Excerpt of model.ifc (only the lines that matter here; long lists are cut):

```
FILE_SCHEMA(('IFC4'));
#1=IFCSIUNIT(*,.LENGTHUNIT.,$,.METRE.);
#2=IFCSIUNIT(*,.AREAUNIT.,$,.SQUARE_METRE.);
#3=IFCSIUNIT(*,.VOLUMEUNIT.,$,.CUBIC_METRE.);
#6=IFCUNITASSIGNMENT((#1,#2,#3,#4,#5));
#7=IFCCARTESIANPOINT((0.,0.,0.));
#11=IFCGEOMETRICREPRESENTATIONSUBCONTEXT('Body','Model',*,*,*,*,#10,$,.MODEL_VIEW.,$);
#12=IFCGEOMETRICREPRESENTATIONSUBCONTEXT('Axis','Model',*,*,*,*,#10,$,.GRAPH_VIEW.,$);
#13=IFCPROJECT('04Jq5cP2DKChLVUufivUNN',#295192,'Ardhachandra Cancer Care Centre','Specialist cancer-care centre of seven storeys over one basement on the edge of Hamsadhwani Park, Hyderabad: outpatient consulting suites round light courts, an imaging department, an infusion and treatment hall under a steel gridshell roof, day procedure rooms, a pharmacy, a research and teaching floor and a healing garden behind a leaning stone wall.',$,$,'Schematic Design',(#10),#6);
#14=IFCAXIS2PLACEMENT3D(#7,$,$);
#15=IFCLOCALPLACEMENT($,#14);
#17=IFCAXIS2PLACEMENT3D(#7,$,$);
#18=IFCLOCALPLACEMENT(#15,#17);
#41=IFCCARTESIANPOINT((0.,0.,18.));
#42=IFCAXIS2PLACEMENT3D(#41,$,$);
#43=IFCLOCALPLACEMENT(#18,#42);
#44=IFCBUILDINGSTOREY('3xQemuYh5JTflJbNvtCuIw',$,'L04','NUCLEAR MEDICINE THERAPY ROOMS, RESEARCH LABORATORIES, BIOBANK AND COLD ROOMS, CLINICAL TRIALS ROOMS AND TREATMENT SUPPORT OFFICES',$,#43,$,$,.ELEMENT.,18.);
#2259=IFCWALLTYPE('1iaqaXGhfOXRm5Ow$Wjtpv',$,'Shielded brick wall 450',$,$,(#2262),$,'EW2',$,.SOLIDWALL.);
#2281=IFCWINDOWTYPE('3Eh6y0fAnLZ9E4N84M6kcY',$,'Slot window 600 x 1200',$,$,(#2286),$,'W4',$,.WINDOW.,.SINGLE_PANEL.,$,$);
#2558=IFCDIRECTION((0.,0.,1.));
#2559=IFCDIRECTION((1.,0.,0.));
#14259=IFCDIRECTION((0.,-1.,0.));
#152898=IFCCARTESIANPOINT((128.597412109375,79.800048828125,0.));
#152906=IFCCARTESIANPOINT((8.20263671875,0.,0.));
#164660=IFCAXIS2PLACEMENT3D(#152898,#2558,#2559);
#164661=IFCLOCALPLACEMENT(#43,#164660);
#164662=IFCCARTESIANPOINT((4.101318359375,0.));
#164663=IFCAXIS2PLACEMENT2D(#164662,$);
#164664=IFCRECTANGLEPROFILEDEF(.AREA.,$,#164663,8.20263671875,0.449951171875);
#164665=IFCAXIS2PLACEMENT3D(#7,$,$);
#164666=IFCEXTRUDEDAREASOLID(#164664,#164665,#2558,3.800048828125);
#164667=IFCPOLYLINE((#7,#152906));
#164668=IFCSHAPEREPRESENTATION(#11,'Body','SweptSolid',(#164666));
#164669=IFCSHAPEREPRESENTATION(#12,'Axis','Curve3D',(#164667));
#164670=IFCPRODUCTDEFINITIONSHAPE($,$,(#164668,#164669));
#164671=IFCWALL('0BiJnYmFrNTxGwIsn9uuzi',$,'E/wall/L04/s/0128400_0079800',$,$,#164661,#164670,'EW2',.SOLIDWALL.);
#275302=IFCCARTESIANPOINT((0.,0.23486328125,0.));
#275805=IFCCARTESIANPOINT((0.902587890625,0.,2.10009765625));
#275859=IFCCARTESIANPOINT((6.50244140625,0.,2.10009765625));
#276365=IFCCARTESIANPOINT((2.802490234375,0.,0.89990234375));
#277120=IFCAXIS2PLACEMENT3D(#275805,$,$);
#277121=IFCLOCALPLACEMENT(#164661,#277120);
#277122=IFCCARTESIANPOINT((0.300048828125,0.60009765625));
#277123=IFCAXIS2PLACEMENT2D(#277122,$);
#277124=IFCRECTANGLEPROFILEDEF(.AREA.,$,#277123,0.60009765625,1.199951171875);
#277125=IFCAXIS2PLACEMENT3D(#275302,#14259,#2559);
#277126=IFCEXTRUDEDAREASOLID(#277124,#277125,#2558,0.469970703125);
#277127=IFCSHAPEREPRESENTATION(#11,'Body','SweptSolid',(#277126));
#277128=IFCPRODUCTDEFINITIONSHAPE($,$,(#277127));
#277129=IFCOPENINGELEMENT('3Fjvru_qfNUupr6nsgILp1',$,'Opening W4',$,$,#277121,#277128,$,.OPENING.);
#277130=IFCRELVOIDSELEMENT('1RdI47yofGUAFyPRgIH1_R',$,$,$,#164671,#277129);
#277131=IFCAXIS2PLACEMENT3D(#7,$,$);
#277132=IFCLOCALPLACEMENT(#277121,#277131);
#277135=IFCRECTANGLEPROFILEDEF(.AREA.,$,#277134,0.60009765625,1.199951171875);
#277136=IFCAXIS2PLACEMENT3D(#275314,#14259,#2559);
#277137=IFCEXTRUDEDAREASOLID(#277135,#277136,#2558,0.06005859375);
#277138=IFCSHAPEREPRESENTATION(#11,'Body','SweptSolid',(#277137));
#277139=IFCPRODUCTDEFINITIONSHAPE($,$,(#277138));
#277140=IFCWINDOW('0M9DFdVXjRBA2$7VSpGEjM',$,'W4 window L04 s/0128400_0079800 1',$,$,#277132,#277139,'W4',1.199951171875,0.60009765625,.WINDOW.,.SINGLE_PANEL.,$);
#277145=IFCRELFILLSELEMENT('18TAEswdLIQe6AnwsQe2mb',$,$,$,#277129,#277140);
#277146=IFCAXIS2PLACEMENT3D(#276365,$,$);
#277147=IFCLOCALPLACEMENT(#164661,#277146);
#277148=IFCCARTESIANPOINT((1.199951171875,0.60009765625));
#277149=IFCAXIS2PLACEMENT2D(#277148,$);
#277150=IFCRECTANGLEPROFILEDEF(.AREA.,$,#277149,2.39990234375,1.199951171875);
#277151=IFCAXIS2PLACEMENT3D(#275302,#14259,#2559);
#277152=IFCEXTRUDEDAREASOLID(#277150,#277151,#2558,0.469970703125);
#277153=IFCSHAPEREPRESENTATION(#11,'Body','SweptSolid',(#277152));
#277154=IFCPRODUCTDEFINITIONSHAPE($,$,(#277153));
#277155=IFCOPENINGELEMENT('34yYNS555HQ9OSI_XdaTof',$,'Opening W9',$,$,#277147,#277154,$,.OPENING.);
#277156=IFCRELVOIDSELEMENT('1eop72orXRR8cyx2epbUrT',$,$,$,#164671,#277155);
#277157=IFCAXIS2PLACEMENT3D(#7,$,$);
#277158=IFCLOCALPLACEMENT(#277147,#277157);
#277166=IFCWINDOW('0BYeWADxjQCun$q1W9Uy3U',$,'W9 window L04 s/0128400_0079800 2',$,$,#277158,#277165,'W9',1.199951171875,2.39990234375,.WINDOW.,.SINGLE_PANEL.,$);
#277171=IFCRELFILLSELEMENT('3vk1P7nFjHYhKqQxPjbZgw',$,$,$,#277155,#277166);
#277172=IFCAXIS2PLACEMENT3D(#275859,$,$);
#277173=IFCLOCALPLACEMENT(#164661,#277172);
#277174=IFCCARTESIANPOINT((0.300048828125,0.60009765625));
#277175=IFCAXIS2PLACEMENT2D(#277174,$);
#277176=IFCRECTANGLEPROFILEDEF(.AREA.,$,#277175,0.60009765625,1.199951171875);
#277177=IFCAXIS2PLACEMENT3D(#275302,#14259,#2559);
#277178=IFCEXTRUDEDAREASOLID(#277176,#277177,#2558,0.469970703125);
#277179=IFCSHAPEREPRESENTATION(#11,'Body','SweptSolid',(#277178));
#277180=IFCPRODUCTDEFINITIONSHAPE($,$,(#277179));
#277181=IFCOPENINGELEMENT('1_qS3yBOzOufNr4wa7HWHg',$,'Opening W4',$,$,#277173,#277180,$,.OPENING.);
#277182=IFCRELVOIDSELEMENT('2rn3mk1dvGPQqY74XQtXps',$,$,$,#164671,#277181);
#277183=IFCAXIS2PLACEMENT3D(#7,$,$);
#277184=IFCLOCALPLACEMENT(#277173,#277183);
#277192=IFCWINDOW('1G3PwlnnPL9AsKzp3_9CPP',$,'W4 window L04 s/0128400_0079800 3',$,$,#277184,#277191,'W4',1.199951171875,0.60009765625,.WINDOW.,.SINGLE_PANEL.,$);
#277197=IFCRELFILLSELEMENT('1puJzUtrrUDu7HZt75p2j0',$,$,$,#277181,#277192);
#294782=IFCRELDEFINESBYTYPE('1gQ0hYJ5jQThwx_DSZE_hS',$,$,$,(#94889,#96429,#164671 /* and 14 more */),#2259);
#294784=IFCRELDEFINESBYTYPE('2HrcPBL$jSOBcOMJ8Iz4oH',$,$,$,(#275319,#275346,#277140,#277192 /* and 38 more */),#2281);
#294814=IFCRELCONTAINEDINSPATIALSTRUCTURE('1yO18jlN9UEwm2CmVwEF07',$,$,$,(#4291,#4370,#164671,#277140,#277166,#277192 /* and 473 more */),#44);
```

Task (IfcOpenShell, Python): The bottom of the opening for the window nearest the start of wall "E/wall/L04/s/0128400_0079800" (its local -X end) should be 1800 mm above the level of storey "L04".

```python
import numpy as np
import ifcopenshell
import ifcopenshell.api.geometry
import ifcopenshell.geom
import ifcopenshell.util.element
import ifcopenshell.util.placement
import ifcopenshell.util.shape
import ifcopenshell.util.unit

model = ifcopenshell.open("model.ifc")
unit_scale = ifcopenshell.util.unit.calculate_unit_scale(model)

window = model.by_guid("0M9DFdVXjRBA2$7VSpGEjM")
opening = window.FillsVoids[0].RelatingOpeningElement
storey = ifcopenshell.util.element.get_container(window, ifc_class="IfcBuildingStorey")
level = ifcopenshell.util.placement.get_local_placement(storey.ObjectPlacement)[2, 3]

# The opening's origin need not be at the sill, so measure its lowest point.
shape = ifcopenshell.geom.create_shape(ifcopenshell.geom.settings(), opening)
bottom = ifcopenshell.util.shape.get_shape_bottom_elevation(shape, shape.geometry) / unit_scale
dz = level + 1.8 / unit_scale - bottom

shift = np.array([0.0, 0.0, dz])
# The window is placed relative to its opening, so it follows when the opening moves.
matrix = ifcopenshell.util.placement.get_local_placement(opening.ObjectPlacement)
matrix[:3, 3] += shift
ifcopenshell.api.geometry.edit_object_placement(
    model, product=opening, matrix=matrix, is_si=False, should_transform_children=True
)

print(f"moved by {dz * unit_scale:+.3f} m")

model.write("model_v2.ifc")
```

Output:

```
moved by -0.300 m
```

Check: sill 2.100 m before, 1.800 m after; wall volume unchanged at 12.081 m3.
